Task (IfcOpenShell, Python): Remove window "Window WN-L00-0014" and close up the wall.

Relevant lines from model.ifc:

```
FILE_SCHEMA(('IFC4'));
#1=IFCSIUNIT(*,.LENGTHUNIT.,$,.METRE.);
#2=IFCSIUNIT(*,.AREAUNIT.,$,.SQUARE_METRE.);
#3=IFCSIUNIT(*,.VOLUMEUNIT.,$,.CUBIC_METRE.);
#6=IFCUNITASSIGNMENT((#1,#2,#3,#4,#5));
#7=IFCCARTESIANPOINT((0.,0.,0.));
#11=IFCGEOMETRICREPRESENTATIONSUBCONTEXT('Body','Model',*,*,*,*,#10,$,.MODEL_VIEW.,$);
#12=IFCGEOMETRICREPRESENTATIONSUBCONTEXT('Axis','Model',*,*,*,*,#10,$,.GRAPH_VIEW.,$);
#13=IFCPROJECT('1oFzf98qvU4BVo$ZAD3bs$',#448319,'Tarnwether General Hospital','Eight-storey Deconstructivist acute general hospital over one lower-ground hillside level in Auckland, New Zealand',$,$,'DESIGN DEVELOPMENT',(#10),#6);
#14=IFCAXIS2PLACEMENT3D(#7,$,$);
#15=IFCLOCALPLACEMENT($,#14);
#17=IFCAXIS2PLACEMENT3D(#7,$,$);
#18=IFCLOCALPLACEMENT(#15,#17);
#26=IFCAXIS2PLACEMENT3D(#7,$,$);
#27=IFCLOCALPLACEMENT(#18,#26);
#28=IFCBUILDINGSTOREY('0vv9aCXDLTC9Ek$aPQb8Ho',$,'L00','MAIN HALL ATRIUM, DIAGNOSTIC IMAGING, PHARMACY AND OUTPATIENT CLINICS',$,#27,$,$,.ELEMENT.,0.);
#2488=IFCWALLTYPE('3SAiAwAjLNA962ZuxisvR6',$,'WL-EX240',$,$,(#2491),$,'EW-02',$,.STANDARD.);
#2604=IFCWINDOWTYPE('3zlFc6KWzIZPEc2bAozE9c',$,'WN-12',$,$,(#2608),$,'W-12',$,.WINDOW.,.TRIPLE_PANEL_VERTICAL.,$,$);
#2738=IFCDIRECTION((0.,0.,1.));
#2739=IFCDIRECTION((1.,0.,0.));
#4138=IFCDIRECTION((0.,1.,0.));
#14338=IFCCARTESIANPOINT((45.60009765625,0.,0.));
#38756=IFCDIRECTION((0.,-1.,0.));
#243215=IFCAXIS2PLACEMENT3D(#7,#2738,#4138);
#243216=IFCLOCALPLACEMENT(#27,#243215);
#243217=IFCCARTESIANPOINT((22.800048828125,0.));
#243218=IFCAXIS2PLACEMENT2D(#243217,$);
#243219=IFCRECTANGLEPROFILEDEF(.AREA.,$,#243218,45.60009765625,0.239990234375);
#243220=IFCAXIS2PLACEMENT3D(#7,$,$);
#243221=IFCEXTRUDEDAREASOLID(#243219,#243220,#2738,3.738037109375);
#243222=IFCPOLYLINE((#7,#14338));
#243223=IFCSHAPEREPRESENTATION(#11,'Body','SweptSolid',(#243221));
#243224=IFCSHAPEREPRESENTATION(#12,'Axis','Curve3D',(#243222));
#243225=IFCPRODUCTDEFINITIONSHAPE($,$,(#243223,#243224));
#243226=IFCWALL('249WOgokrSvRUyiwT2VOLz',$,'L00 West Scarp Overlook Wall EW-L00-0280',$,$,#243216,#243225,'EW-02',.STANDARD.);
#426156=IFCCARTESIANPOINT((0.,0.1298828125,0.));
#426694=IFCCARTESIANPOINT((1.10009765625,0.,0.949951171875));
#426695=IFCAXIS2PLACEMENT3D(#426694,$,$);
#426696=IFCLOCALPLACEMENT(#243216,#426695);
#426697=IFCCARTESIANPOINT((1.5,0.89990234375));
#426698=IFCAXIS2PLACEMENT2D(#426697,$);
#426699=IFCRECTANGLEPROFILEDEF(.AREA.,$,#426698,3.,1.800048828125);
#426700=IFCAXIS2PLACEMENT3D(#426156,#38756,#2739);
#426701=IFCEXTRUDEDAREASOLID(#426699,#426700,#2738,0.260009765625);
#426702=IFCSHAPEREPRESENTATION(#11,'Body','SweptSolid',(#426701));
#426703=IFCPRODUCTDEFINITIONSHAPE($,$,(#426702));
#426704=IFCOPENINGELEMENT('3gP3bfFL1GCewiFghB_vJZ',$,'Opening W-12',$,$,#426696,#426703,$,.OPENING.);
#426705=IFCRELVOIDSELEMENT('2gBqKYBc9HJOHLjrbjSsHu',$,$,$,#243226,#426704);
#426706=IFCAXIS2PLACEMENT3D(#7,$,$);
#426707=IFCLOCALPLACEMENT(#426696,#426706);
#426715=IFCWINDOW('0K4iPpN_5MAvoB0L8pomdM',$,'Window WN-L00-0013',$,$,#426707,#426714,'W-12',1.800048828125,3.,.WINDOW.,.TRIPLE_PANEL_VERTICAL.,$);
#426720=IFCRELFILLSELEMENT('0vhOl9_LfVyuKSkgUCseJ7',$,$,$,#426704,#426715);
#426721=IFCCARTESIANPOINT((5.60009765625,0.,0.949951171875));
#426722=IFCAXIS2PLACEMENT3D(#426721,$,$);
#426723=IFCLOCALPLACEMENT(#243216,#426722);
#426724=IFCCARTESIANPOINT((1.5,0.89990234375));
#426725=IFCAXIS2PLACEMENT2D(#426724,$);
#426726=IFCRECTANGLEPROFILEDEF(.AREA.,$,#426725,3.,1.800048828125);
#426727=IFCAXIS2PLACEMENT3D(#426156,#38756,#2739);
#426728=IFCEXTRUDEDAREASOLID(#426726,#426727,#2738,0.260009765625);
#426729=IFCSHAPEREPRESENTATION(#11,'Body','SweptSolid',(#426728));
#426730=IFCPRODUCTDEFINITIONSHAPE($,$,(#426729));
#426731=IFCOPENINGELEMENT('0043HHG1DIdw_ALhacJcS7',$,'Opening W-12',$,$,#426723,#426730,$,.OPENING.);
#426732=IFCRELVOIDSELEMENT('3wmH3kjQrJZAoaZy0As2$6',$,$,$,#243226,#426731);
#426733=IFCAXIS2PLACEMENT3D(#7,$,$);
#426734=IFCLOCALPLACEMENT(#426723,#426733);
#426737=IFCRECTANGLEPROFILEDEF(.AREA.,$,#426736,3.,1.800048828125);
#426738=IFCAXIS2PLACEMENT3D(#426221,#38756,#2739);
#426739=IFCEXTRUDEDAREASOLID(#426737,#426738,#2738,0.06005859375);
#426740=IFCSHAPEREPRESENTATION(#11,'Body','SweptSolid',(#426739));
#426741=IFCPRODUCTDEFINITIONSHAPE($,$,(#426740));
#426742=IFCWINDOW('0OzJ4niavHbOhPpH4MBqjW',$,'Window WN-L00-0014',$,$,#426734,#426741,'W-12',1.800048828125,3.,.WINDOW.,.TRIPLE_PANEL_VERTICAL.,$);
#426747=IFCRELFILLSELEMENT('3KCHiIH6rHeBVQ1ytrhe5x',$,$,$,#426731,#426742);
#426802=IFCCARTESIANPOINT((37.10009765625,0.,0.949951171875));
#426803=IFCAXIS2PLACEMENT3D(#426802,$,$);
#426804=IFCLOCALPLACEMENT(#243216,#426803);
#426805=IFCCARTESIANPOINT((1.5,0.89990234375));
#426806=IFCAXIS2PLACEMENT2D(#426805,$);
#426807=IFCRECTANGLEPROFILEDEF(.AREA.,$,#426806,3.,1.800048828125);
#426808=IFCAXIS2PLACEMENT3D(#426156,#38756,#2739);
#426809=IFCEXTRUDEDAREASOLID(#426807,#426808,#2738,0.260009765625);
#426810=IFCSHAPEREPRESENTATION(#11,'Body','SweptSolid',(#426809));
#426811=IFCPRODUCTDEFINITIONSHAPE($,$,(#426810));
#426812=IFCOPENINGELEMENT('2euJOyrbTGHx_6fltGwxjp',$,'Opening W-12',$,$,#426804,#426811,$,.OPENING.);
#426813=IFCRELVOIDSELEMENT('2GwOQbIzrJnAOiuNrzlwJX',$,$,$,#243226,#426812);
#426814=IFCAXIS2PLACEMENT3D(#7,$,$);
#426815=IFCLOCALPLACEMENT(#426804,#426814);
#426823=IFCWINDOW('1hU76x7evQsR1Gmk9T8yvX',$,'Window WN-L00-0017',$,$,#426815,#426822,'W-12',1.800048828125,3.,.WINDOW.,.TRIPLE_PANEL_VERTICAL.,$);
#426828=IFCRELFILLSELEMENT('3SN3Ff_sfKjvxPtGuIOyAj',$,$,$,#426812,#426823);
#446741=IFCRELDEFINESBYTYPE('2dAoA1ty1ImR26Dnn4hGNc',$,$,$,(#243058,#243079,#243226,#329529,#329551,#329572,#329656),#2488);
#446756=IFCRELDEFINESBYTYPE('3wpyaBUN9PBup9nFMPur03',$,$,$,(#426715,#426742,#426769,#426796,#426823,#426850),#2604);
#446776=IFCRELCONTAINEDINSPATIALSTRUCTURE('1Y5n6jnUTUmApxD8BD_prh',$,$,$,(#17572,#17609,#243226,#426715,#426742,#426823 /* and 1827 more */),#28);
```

```python
import ifcopenshell
import ifcopenshell.api.feature
import ifcopenshell.api.root
import ifcopenshell.geom
import ifcopenshell.util.shape

model = ifcopenshell.open("model.ifc")
settings = ifcopenshell.geom.settings()


def volume(element):
    """Net volume in cubic metres, openings subtracted."""
    shape = ifcopenshell.geom.create_shape(settings, element)
    return ifcopenshell.util.shape.get_volume(shape.geometry)


window = model.by_id(426742)
opening = window.FillsVoids[0].RelatingOpeningElement
wall = opening.VoidsElements[0].RelatingBuildingElement
before = volume(wall)

ifcopenshell.api.root.remove_product(model, product=window)
ifcopenshell.api.feature.remove_feature(model, feature=opening)

after = volume(wall)

print(f"wall volume {before:.3f} -> {after:.3f} m3")

model.write("model_edited.ifc")
```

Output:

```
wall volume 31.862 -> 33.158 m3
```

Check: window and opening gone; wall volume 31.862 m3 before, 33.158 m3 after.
